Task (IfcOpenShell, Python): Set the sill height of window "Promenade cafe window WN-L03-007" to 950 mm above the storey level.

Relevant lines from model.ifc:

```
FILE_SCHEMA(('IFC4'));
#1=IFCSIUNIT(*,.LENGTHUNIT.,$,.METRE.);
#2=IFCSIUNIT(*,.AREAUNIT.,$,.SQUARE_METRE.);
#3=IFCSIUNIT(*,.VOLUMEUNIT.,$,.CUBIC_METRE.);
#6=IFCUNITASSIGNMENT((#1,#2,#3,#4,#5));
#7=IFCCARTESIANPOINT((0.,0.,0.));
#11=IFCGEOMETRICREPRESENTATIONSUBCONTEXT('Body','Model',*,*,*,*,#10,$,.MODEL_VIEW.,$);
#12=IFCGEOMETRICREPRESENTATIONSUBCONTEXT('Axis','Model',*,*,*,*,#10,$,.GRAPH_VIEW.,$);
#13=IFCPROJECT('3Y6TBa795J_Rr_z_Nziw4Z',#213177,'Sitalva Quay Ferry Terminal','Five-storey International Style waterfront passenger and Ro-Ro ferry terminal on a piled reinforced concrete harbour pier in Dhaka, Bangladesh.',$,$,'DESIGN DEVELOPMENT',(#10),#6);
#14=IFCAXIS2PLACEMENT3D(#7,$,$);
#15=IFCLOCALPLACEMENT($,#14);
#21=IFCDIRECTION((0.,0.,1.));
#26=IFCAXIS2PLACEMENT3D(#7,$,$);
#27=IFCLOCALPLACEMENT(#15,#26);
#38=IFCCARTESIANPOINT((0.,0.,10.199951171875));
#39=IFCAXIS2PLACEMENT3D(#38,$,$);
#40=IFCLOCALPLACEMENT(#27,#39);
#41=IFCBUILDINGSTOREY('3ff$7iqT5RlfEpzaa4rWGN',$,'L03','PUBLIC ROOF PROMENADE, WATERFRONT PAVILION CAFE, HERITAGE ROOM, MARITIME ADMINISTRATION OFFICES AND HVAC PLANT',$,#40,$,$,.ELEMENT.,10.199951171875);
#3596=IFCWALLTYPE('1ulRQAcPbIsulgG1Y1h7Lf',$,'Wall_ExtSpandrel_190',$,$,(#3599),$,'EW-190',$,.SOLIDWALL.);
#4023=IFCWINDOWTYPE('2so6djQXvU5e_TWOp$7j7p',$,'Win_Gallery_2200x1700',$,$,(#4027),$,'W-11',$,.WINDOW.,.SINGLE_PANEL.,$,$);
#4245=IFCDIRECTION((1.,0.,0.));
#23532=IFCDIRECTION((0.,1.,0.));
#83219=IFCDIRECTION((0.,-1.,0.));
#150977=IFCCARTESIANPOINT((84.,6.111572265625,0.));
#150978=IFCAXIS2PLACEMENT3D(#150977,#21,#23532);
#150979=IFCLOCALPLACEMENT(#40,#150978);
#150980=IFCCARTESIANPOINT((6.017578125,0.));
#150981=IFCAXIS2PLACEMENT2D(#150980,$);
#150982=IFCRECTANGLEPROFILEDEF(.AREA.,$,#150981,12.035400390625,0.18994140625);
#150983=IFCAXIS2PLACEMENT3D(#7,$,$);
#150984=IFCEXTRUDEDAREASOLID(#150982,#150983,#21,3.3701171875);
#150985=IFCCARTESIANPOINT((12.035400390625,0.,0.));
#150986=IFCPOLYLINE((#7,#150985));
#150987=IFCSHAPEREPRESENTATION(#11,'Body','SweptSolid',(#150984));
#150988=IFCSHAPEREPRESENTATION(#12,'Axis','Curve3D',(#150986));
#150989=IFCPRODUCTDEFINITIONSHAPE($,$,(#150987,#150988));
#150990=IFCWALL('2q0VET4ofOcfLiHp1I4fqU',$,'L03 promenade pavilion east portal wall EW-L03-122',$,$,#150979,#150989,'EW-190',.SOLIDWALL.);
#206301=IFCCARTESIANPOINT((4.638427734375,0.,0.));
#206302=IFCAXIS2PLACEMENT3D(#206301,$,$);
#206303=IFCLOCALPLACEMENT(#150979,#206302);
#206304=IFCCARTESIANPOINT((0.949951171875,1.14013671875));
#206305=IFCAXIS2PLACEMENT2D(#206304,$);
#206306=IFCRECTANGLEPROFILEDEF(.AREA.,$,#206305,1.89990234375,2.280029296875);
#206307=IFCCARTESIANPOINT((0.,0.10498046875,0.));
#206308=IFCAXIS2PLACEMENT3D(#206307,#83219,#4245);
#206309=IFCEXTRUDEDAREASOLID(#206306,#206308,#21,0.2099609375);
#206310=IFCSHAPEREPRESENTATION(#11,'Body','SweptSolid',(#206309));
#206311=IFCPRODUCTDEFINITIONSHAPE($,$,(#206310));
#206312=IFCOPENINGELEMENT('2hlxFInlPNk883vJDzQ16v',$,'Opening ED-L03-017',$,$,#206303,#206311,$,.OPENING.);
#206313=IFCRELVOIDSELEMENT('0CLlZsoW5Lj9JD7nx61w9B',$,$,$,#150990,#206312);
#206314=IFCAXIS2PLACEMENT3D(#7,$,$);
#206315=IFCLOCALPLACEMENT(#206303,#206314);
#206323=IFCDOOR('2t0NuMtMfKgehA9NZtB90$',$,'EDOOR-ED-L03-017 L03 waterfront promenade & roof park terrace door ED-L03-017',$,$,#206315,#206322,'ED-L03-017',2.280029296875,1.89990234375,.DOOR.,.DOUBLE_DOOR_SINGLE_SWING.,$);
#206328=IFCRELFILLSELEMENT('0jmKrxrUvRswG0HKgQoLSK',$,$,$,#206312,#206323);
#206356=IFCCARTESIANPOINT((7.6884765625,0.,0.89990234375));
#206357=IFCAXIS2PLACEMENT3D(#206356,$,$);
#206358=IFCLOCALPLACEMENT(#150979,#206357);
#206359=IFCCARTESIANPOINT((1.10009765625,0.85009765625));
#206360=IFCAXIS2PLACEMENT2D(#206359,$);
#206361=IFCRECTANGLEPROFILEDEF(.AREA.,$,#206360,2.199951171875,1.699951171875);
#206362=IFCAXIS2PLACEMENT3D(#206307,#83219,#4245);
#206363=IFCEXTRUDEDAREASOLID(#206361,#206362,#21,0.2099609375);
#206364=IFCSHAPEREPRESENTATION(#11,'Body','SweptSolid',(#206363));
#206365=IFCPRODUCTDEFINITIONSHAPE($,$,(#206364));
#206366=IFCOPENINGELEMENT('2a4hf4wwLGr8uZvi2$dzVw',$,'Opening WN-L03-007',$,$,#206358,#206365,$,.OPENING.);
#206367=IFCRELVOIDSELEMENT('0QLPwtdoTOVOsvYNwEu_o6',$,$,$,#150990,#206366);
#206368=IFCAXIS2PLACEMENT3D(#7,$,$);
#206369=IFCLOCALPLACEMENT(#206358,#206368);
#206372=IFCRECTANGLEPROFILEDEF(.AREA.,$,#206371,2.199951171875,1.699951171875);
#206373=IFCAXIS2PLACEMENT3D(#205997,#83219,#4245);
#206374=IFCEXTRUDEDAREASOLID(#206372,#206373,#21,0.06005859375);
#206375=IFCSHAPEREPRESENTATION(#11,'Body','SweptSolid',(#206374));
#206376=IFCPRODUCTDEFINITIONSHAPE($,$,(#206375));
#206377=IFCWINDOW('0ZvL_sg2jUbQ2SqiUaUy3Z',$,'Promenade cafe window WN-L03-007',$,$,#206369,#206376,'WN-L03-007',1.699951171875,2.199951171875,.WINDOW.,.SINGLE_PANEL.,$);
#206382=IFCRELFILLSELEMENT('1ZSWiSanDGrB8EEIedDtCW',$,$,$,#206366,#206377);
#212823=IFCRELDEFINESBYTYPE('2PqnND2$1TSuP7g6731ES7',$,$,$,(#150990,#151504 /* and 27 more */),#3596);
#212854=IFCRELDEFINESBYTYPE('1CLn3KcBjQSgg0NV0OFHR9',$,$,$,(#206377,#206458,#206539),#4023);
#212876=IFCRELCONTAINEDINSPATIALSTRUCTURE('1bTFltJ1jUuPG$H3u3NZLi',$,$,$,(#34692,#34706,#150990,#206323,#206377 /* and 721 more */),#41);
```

```python
import numpy as np
import ifcopenshell
import ifcopenshell.api.geometry
import ifcopenshell.geom
import ifcopenshell.util.element
import ifcopenshell.util.placement
import ifcopenshell.util.shape
import ifcopenshell.util.unit

model = ifcopenshell.open("model.ifc")
unit_scale = ifcopenshell.util.unit.calculate_unit_scale(model)

window = model.by_id(206377)
opening = window.FillsVoids[0].RelatingOpeningElement
storey = ifcopenshell.util.element.get_container(window, ifc_class="IfcBuildingStorey")
level = ifcopenshell.util.placement.get_local_placement(storey.ObjectPlacement)[2, 3]

# The opening's origin need not be at the sill, so measure its lowest point.
shape = ifcopenshell.geom.create_shape(ifcopenshell.geom.settings(), opening)
bottom = ifcopenshell.util.shape.get_shape_bottom_elevation(shape, shape.geometry) / unit_scale
dz = level + 0.95 / unit_scale - bottom

shift = np.array([0.0, 0.0, dz])
# The window is placed relative to its opening, so it follows when the opening moves.
matrix = ifcopenshell.util.placement.get_local_placement(opening.ObjectPlacement)
matrix[:3, 3] += shift
ifcopenshell.api.geometry.edit_object_placement(
    model, product=opening, matrix=matrix, is_si=False, should_transform_children=True
)

print(f"moved by {dz * unit_scale:+.3f} m")

model.write("model_edited.ifc")
```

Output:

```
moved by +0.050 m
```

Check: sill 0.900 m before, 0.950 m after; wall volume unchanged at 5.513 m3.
